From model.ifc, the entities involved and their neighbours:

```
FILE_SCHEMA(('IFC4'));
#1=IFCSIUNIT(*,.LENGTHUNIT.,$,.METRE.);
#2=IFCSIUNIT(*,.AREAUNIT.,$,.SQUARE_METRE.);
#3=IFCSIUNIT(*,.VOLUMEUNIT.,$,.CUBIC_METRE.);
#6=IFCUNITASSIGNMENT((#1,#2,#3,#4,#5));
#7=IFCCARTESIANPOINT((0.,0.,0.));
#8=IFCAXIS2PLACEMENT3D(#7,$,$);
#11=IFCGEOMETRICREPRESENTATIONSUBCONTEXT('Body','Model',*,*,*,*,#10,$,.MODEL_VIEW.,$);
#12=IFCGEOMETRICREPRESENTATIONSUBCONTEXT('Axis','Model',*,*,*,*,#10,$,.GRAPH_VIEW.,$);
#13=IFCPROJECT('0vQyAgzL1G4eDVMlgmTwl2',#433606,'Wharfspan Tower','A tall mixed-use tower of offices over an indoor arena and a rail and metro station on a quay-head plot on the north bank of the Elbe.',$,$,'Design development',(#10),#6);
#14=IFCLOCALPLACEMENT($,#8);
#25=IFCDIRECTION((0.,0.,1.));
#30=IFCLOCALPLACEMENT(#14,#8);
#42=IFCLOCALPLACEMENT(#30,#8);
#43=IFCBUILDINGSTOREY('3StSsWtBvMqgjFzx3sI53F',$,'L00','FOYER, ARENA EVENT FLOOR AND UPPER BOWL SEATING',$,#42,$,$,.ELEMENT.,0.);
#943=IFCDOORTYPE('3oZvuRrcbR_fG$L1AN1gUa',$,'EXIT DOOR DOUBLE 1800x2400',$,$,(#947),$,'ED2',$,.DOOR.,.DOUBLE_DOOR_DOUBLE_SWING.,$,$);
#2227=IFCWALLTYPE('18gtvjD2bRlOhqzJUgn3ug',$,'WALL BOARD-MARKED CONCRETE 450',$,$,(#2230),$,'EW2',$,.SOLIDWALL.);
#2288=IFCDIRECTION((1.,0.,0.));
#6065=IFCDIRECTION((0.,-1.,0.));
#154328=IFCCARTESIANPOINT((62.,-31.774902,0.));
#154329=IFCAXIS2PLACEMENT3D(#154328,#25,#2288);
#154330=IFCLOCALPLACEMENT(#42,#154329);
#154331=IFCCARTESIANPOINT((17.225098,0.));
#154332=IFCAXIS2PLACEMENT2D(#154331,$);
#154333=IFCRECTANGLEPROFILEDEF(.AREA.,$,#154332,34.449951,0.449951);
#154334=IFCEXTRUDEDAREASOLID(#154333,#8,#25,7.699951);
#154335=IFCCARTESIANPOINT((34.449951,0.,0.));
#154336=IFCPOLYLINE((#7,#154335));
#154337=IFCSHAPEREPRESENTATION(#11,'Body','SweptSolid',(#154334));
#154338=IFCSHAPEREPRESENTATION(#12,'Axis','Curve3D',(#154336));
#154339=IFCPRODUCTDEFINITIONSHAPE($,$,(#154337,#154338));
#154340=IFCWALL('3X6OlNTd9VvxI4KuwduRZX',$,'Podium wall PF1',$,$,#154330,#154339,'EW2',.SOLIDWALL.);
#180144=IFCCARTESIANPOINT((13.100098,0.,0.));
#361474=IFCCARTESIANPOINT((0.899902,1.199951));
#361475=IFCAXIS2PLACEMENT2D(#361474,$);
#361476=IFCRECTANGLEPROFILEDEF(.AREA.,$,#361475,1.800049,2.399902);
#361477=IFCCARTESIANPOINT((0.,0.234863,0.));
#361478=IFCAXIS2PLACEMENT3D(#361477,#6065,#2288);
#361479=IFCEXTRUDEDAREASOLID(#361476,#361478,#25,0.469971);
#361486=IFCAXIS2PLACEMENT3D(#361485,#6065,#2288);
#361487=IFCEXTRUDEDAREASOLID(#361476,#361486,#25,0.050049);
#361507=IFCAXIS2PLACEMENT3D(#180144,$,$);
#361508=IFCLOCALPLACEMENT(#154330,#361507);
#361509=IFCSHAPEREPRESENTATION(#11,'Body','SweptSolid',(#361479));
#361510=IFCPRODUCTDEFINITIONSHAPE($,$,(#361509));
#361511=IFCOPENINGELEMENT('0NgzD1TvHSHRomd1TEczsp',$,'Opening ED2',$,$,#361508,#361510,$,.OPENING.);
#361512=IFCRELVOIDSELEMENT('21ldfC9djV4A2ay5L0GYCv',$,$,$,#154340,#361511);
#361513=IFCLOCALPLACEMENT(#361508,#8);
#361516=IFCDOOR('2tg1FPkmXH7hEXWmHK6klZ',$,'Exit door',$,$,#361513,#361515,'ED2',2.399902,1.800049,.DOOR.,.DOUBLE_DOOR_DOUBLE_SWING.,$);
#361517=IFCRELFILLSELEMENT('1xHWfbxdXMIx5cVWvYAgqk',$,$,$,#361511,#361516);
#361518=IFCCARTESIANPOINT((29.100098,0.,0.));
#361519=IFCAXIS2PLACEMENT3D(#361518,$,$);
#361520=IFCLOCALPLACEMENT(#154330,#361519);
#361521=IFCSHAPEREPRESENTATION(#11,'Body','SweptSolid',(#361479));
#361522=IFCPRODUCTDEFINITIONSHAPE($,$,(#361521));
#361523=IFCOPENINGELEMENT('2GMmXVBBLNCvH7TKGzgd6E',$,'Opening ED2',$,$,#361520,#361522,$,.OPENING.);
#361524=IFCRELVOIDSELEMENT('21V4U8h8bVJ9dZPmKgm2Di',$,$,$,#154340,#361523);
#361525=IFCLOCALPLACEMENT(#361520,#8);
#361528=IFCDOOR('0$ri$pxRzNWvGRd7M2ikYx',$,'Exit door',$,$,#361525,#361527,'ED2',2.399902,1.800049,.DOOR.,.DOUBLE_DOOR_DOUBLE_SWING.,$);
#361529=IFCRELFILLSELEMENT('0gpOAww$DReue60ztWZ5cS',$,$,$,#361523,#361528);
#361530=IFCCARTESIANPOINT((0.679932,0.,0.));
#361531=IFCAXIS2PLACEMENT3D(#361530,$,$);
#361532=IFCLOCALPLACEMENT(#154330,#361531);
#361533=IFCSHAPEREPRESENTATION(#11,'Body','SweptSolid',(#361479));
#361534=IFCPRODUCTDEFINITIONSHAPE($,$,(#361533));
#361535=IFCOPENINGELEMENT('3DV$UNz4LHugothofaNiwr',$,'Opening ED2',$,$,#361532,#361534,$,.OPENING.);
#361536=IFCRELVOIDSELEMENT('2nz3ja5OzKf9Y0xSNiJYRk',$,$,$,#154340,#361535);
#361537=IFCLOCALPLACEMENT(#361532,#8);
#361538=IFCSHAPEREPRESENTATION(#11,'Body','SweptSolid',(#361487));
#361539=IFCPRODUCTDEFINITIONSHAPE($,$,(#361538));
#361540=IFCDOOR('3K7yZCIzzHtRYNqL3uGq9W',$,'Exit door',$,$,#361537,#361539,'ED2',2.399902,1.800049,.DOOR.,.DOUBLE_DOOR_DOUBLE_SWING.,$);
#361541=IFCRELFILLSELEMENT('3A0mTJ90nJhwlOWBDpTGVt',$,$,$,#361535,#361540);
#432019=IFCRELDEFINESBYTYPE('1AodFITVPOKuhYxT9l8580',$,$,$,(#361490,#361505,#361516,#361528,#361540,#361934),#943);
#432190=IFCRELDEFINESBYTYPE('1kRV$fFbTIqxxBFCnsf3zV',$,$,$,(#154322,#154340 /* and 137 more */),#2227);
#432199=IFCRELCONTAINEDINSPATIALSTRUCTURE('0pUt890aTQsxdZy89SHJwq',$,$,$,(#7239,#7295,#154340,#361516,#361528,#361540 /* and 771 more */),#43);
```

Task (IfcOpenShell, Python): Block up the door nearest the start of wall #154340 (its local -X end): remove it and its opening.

```python
import ifcopenshell
import ifcopenshell.api.feature
import ifcopenshell.api.root
import ifcopenshell.geom
import ifcopenshell.util.shape

model = ifcopenshell.open("model.ifc")
settings = ifcopenshell.geom.settings()


def volume(element):
    """Net volume in cubic metres, openings subtracted."""
    shape = ifcopenshell.geom.create_shape(settings, element)
    return ifcopenshell.util.shape.get_volume(shape.geometry)


door = model.by_guid("3K7yZCIzzHtRYNqL3uGq9W")
opening = door.FillsVoids[0].RelatingOpeningElement
wall = opening.VoidsElements[0].RelatingBuildingElement
before = volume(wall)

ifcopenshell.api.root.remove_product(model, product=door)
ifcopenshell.api.feature.remove_feature(model, feature=opening)

after = volume(wall)

print(f"wall volume {before:.3f} -> {after:.3f} m3")

model.write("model-out.ifc")
```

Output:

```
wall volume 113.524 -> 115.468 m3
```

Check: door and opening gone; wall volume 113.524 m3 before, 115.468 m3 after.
